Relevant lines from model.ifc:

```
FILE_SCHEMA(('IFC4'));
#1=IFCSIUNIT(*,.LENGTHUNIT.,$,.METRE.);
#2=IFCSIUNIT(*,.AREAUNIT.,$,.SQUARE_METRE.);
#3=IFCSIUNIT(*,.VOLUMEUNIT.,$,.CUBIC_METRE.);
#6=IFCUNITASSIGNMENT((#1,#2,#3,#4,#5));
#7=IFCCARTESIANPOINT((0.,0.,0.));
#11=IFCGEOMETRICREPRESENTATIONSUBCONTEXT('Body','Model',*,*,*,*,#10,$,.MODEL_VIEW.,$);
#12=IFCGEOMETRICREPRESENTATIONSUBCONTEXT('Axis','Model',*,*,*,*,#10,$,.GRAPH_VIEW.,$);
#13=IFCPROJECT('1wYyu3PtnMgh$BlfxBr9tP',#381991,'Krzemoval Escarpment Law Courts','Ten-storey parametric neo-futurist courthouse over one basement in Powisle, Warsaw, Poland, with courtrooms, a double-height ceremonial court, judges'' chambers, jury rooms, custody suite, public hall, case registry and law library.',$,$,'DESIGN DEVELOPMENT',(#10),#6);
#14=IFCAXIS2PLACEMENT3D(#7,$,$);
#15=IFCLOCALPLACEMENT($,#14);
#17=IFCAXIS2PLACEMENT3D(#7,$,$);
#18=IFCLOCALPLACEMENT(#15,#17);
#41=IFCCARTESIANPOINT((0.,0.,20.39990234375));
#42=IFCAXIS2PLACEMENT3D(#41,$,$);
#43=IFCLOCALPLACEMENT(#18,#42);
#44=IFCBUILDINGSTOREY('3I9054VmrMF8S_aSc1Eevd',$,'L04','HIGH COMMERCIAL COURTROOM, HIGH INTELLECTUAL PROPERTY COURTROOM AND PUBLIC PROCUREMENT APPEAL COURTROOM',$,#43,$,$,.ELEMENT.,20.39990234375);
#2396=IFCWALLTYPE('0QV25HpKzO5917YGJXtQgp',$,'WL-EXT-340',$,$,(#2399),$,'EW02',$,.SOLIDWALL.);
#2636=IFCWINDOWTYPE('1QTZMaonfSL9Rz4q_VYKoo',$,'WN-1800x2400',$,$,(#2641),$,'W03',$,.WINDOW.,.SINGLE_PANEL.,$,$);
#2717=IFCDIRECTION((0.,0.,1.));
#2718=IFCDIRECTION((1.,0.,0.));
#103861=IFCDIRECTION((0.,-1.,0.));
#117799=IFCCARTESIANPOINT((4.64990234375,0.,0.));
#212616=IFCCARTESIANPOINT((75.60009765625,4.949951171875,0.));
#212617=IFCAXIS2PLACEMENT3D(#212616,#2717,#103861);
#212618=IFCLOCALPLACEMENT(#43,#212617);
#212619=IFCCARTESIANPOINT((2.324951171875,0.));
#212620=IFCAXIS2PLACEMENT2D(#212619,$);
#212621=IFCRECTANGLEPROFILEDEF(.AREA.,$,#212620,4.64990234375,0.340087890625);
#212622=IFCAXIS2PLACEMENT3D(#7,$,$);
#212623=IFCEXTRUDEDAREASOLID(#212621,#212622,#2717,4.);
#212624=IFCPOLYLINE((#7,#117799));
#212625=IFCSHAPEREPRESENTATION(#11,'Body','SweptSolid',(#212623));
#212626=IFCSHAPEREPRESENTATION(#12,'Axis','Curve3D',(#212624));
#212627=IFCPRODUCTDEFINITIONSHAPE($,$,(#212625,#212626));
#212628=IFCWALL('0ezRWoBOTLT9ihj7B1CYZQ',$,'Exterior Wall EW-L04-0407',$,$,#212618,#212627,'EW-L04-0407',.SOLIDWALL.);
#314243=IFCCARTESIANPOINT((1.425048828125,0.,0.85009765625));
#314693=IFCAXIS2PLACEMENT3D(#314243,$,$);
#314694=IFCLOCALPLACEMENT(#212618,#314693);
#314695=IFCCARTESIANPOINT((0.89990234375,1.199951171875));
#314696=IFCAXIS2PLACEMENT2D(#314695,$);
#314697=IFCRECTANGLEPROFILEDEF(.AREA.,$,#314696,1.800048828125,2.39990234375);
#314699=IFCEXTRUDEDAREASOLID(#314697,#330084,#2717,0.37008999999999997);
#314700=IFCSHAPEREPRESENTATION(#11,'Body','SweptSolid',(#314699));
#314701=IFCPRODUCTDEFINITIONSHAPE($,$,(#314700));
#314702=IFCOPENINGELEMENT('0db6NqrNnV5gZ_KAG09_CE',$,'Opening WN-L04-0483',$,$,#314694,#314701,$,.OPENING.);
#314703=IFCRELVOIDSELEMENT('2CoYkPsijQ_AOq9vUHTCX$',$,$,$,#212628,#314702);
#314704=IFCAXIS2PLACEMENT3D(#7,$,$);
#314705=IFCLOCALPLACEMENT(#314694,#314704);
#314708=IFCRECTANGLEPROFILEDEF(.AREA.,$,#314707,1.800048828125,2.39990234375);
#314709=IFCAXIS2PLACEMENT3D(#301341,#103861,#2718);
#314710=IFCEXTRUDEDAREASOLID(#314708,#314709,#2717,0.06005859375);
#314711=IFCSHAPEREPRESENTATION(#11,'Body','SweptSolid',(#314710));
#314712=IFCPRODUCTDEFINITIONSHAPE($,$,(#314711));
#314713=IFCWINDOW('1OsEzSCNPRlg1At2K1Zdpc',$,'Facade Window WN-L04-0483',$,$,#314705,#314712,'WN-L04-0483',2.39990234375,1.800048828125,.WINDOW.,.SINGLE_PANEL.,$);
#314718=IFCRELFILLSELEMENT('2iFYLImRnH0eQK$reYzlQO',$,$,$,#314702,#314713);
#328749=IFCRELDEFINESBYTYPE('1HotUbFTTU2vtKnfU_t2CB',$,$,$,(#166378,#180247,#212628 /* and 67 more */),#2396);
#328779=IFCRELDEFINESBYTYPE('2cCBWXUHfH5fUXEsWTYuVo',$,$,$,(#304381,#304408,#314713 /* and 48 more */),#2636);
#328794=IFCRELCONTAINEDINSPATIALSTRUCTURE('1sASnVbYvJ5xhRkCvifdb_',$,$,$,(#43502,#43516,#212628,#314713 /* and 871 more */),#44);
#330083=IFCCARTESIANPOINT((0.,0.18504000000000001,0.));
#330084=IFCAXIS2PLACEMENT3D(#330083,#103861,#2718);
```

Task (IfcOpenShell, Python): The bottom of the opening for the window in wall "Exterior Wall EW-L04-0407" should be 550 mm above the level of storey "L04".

```python
import numpy as np
import ifcopenshell
import ifcopenshell.api.geometry
import ifcopenshell.geom
import ifcopenshell.util.element
import ifcopenshell.util.placement
import ifcopenshell.util.shape
import ifcopenshell.util.unit

model = ifcopenshell.open("model.ifc")
unit_scale = ifcopenshell.util.unit.calculate_unit_scale(model)

window = model.by_guid("1OsEzSCNPRlg1At2K1Zdpc")
opening = window.FillsVoids[0].RelatingOpeningElement
storey = ifcopenshell.util.element.get_container(window, ifc_class="IfcBuildingStorey")
level = ifcopenshell.util.placement.get_local_placement(storey.ObjectPlacement)[2, 3]

# The opening's origin need not be at the sill, so measure its lowest point.
shape = ifcopenshell.geom.create_shape(ifcopenshell.geom.settings(), opening)
bottom = ifcopenshell.util.shape.get_shape_bottom_elevation(shape, shape.geometry) / unit_scale
dz = level + 0.55 / unit_scale - bottom

shift = np.array([0.0, 0.0, dz])
# The window is placed relative to its opening, so it follows when the opening moves.
matrix = ifcopenshell.util.placement.get_local_placement(opening.ObjectPlacement)
matrix[:3, 3] += shift
ifcopenshell.api.geometry.edit_object_placement(
    model, product=opening, matrix=matrix, is_si=False, should_transform_children=True
)

print(f"moved by {dz * unit_scale:+.3f} m")

model.write("model-out.ifc")
```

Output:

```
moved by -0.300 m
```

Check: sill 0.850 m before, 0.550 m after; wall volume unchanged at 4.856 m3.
